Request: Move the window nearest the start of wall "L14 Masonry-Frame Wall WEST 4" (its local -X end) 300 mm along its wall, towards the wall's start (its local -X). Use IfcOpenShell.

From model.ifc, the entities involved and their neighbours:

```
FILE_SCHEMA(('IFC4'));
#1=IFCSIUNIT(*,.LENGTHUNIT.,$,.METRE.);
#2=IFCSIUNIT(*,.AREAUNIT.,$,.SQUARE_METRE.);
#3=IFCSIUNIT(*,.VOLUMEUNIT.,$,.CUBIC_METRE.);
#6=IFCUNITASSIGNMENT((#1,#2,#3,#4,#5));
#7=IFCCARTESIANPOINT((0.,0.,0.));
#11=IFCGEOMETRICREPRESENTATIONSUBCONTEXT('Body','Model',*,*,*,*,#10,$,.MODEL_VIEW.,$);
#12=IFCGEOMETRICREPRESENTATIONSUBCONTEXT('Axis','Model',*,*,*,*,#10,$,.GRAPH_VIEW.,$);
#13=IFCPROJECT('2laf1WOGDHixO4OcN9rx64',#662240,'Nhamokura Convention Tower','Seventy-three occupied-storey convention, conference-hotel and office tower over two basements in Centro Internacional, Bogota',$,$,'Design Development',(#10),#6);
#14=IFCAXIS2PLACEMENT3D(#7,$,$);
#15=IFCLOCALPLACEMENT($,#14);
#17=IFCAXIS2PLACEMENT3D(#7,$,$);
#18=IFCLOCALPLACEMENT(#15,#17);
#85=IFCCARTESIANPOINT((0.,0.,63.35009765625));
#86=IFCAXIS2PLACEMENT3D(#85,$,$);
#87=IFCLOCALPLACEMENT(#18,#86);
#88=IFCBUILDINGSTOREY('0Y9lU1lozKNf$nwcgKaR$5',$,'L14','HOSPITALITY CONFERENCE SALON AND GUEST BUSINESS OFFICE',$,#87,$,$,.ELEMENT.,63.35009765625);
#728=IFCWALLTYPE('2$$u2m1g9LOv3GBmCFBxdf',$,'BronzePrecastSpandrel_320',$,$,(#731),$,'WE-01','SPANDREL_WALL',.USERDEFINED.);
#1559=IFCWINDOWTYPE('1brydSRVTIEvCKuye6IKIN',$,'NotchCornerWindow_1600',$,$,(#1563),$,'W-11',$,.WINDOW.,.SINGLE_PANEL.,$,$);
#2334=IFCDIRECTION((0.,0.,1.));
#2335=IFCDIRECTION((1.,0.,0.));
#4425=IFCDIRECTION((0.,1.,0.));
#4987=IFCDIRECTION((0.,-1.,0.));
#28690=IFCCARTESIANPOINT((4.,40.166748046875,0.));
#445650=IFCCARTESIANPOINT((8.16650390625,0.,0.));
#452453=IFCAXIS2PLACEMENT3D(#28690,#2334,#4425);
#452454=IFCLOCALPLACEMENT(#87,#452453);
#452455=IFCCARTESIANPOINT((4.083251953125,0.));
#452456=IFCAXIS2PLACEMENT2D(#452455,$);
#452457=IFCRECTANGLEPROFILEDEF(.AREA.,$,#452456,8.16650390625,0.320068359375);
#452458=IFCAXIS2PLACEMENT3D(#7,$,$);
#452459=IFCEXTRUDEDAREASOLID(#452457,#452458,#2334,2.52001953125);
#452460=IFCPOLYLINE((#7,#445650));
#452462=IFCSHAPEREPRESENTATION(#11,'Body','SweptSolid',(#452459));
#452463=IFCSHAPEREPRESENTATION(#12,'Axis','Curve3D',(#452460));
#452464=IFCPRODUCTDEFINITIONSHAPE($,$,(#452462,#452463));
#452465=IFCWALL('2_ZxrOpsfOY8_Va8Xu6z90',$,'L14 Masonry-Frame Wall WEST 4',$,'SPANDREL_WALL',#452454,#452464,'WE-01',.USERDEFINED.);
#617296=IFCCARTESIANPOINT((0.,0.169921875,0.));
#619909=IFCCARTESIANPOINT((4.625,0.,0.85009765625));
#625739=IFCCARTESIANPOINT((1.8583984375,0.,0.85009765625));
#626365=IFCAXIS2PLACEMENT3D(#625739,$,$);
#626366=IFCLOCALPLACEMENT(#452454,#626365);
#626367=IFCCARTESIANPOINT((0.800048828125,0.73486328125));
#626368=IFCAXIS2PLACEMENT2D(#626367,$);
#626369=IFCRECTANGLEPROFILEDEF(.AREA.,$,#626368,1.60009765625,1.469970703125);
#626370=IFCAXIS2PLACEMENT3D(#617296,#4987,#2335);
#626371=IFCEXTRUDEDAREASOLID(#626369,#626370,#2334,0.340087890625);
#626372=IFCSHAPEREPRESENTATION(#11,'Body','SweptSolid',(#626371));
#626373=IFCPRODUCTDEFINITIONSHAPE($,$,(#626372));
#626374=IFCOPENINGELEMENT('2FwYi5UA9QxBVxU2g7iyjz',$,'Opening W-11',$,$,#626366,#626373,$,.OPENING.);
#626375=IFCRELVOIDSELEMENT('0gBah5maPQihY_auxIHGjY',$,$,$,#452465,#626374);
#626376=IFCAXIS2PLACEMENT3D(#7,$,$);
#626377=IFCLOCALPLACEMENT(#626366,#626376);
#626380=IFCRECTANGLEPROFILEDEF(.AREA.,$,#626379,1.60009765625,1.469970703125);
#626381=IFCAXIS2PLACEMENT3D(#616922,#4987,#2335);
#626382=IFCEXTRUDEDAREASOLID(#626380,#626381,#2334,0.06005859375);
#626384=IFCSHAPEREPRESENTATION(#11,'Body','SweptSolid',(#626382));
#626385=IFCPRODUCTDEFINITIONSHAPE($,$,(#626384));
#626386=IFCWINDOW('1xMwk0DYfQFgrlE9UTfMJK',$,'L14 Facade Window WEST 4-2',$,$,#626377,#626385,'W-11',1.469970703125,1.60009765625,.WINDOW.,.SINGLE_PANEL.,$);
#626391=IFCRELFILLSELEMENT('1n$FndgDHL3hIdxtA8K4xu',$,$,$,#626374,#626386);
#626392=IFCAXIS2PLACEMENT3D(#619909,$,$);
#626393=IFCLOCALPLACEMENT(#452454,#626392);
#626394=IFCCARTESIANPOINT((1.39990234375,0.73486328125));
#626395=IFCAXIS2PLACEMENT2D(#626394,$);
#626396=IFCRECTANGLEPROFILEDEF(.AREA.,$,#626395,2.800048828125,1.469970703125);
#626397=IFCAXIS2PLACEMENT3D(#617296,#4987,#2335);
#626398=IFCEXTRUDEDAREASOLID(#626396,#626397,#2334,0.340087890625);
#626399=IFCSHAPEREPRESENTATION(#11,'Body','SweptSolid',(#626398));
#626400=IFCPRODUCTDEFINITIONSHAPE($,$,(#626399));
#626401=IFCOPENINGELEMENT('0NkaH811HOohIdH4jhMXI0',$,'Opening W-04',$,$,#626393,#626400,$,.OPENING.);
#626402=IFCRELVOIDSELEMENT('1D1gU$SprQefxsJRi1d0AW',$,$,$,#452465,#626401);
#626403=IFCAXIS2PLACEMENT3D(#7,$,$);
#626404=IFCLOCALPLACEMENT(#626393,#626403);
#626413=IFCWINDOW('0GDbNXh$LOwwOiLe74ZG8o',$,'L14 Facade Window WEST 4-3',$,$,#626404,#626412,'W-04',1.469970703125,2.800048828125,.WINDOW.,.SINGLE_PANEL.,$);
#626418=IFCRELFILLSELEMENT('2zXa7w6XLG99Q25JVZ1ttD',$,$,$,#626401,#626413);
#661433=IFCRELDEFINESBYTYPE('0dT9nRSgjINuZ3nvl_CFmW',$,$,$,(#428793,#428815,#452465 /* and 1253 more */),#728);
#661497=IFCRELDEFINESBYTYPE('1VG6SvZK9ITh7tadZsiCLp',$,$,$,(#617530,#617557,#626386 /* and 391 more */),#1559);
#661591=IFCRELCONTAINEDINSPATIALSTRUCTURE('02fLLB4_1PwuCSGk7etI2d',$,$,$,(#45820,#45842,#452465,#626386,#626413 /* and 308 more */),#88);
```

```python
import ifcopenshell
import ifcopenshell.api.geometry
import ifcopenshell.util.placement
import ifcopenshell.util.unit

model = ifcopenshell.open("model.ifc")
unit_scale = ifcopenshell.util.unit.calculate_unit_scale(model)

window = model.by_guid("1xMwk0DYfQFgrlE9UTfMJK")
opening = window.FillsVoids[0].RelatingOpeningElement
wall = opening.VoidsElements[0].RelatingBuildingElement

wall_matrix = ifcopenshell.util.placement.get_local_placement(wall.ObjectPlacement)
shift = wall_matrix[:3, 0] * -0.3 / unit_scale
before = ifcopenshell.util.placement.get_local_placement(window.ObjectPlacement)[:3, 3].copy()

# The window is placed relative to its opening, so it follows when the opening moves.
matrix = ifcopenshell.util.placement.get_local_placement(opening.ObjectPlacement)
matrix[:3, 3] += shift
ifcopenshell.api.geometry.edit_object_placement(
    model, product=opening, matrix=matrix, is_si=False, should_transform_children=True
)

after = ifcopenshell.util.placement.get_local_placement(window.ObjectPlacement)[:3, 3]
print("window moved by", (after - before).round(3) + 0.0)

model.write("model_v2.ifc")
```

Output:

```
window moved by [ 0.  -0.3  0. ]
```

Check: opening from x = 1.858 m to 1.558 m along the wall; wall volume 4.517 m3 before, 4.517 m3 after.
